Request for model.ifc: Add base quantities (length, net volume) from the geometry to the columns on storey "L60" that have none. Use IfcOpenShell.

First a look at what the model holds.

```python
import ifcopenshell
import ifcopenshell.util.element
import ifcopenshell.util.unit

model = ifcopenshell.open("model.ifc")
print(model.schema)
for unit_type in ("LENGTHUNIT", "AREAUNIT", "VOLUMEUNIT"):
    print(unit_type, ifcopenshell.util.unit.calculate_unit_scale(model, unit_type))
storey = next(s for s in model.by_type("IfcBuildingStorey") if s.Name == "L60")
columns = [e for e in ifcopenshell.util.element.get_decomposition(storey) if e.is_a("IfcColumn")]
for e in sorted(columns, key=lambda e: e.id()):
    print(e.id(), e.is_a(), e.Name, list(ifcopenshell.util.element.get_psets(e, qtos_only=True)), sep=" | ")
```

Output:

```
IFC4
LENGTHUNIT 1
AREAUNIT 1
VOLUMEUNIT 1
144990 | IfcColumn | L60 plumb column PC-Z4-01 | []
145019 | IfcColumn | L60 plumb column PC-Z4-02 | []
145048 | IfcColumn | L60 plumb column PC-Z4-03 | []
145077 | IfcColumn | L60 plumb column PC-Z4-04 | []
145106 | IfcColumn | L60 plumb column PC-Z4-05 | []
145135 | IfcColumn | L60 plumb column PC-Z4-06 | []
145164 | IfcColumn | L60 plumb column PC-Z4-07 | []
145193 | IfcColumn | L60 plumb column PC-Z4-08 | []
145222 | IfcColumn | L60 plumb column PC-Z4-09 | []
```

```python
import ifcopenshell
import ifcopenshell.api.pset
import ifcopenshell.geom
import ifcopenshell.util.element
import ifcopenshell.util.shape
import ifcopenshell.util.unit

model = ifcopenshell.open("model.ifc")
unit_scale = ifcopenshell.util.unit.calculate_unit_scale(model)
volume_scale = ifcopenshell.util.unit.calculate_unit_scale(model, "VOLUMEUNIT")
settings = ifcopenshell.geom.settings()

storey = next(s for s in model.by_type("IfcBuildingStorey") if s.Name == "L60")
columns = [e for e in ifcopenshell.util.element.get_decomposition(storey) if e.is_a("IfcColumn")]

for e in sorted(columns, key=lambda e: e.id()):
    if ifcopenshell.util.element.get_psets(e, qtos_only=True, should_inherit=False):
        continue
    # Geometry comes back in metres, in the element's own axes.
    shape = ifcopenshell.geom.create_shape(settings, e)
    values = {
        "Length": ifcopenshell.util.shape.get_z(shape.geometry) / unit_scale,
        "NetVolume": ifcopenshell.util.shape.get_volume(shape.geometry) / volume_scale,
    }
    qto = ifcopenshell.api.pset.add_qto(model, product=e, name="Qto_ColumnBaseQuantities")
    ifcopenshell.api.pset.edit_qto(model, qto=qto, properties=values)
    print(e.id(), {k: round(v, 3) for k, v in values.items()})

model.write("model-out.ifc")
```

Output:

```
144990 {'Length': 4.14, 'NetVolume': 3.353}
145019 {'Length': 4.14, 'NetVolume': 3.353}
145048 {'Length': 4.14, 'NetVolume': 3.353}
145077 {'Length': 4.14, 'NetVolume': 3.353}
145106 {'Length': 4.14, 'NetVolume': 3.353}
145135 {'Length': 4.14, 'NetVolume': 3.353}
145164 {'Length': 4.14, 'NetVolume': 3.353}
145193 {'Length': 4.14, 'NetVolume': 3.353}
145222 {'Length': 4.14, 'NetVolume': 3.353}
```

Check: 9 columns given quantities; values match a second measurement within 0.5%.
